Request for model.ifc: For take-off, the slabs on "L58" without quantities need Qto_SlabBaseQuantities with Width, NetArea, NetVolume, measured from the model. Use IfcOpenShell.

First a look at what the model holds.

```python
import ifcopenshell
import ifcopenshell.util.element
import ifcopenshell.util.unit

model = ifcopenshell.open("model.ifc")
print(model.schema)
for unit_type in ("LENGTHUNIT", "AREAUNIT", "VOLUMEUNIT"):
    print(unit_type, ifcopenshell.util.unit.calculate_unit_scale(model, unit_type))
storey = next(s for s in model.by_type("IfcBuildingStorey") if s.Name == "L58")
slabs = [e for e in ifcopenshell.util.element.get_decomposition(storey) if e.is_a("IfcSlab")]
for e in sorted(slabs, key=lambda e: e.id()):
    print(e.id(), e.is_a(), e.Name, list(ifcopenshell.util.element.get_psets(e, qtos_only=True)), sep=" | ")
```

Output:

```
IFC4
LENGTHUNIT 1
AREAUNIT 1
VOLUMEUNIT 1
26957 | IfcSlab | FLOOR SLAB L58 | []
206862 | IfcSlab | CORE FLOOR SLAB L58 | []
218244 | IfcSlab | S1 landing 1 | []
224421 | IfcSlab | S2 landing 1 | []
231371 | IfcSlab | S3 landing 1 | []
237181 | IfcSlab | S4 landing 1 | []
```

```python
import ifcopenshell
import ifcopenshell.api.pset
import ifcopenshell.geom
import ifcopenshell.util.element
import ifcopenshell.util.shape
import ifcopenshell.util.unit

model = ifcopenshell.open("model.ifc")
unit_scale = ifcopenshell.util.unit.calculate_unit_scale(model)
area_scale = ifcopenshell.util.unit.calculate_unit_scale(model, "AREAUNIT")
volume_scale = ifcopenshell.util.unit.calculate_unit_scale(model, "VOLUMEUNIT")
settings = ifcopenshell.geom.settings()

storey = next(s for s in model.by_type("IfcBuildingStorey") if s.Name == "L58")
slabs = [e for e in ifcopenshell.util.element.get_decomposition(storey) if e.is_a("IfcSlab")]

for e in sorted(slabs, key=lambda e: e.id()):
    if ifcopenshell.util.element.get_psets(e, qtos_only=True, should_inherit=False):
        continue
    # Geometry comes back in metres, in the element's own axes.
    shape = ifcopenshell.geom.create_shape(settings, e)
    values = {
        "Width": ifcopenshell.util.shape.get_z(shape.geometry) / unit_scale,
        "NetArea": ifcopenshell.util.shape.get_footprint_area(shape.geometry) / area_scale,
        "NetVolume": ifcopenshell.util.shape.get_volume(shape.geometry) / volume_scale,
    }
    qto = ifcopenshell.api.pset.add_qto(model, product=e, name="Qto_SlabBaseQuantities")
    ifcopenshell.api.pset.edit_qto(model, qto=qto, properties=values)
    print(e.id(), {k: round(v, 3) for k, v in values.items()})

model.write("model_edited.ifc")
```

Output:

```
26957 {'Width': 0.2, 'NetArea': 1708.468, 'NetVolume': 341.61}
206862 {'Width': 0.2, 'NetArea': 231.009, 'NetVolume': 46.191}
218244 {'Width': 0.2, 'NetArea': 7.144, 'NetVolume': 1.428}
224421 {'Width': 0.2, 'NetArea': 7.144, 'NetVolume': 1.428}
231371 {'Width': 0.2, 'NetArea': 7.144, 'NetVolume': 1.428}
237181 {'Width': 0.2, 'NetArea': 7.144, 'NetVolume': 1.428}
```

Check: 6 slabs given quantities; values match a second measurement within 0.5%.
